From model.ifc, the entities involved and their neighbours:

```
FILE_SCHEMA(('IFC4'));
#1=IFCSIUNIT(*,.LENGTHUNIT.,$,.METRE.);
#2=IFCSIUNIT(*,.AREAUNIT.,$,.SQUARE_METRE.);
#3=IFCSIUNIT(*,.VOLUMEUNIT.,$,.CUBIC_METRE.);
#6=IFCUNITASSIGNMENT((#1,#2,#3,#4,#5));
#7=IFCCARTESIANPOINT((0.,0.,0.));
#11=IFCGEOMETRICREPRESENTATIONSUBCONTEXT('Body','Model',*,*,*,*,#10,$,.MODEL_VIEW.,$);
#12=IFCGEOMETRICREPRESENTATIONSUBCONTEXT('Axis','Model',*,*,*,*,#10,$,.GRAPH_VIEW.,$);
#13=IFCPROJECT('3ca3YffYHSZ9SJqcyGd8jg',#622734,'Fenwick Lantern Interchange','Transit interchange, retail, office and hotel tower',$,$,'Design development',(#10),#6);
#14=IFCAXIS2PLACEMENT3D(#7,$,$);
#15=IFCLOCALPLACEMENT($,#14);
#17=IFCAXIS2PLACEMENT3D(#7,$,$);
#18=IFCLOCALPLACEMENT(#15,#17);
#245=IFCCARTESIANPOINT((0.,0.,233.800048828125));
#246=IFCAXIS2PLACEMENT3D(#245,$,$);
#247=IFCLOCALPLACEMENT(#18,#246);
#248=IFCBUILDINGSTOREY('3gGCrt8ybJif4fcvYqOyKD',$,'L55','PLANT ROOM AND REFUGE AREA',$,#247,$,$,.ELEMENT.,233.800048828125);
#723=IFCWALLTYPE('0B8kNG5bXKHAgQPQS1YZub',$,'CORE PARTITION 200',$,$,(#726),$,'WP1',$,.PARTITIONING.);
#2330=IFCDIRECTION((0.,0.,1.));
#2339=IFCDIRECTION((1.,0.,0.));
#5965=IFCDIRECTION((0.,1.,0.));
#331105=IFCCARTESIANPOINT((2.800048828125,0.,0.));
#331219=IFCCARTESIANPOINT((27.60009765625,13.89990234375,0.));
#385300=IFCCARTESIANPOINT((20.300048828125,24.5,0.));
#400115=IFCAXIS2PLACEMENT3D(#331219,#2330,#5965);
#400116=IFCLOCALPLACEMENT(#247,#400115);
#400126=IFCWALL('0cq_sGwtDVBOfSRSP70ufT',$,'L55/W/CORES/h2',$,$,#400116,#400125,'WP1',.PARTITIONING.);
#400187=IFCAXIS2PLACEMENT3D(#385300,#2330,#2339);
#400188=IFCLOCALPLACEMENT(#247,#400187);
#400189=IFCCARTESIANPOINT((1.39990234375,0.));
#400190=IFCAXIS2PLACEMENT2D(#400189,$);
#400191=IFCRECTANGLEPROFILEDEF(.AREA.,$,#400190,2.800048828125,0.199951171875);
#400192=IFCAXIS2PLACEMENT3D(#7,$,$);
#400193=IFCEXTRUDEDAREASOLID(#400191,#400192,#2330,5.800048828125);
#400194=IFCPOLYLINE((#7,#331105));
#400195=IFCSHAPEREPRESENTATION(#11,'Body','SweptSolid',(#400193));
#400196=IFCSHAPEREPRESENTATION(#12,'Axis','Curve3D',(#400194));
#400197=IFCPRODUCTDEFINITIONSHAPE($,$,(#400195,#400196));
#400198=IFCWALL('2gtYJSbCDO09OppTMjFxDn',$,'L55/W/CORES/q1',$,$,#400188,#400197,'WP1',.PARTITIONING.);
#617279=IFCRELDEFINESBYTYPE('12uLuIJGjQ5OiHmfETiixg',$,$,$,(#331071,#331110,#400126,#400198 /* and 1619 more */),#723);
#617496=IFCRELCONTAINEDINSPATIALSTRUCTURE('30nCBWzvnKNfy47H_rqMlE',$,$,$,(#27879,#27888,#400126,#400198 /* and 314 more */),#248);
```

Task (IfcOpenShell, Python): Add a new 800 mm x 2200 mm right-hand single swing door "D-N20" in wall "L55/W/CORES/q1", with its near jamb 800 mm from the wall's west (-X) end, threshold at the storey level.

```python
import numpy as np
import ifcopenshell
import ifcopenshell.api.feature
import ifcopenshell.api.geometry
import ifcopenshell.api.root
import ifcopenshell.api.spatial
import ifcopenshell.geom
import ifcopenshell.util.element
import ifcopenshell.util.placement
import ifcopenshell.util.representation
import ifcopenshell.util.shape
import ifcopenshell.util.unit

model = ifcopenshell.open("model.ifc")
unit_scale = ifcopenshell.util.unit.calculate_unit_scale(model)
settings = ifcopenshell.geom.settings()


def volume(element):
    """Net volume in cubic metres, openings subtracted."""
    shape = ifcopenshell.geom.create_shape(settings, element)
    return ifcopenshell.util.shape.get_volume(shape.geometry)


wall = model.by_guid("2gtYJSbCDO09OppTMjFxDn")
storey = ifcopenshell.util.element.get_container(wall, ifc_class="IfcBuildingStorey")
context = ifcopenshell.util.representation.get_context(model, "Model", "Body", "MODEL_VIEW")
before = volume(wall)

width, height, from_end, sill = 0.8, 2.2, 0.8, 0.0  # metres

# The wall runs along its own X axis, and the end named is its -X end.
wall_shape = ifcopenshell.geom.create_shape(settings, wall)
x, y, z = ifcopenshell.util.shape.get_vertices(wall_shape.geometry).T
start = x.min() + from_end
face, thickness = float(y.min()), float(y.max() - y.min())
wall_matrix = ifcopenshell.util.placement.get_local_placement(wall.ObjectPlacement)
level = ifcopenshell.util.placement.get_local_placement(storey.ObjectPlacement)[2, 3]


def in_wall(x, y):
    """Placement at x, y metres in the wall's axes, at sill height."""
    matrix = wall_matrix.copy()
    matrix[:, 3] = wall_matrix @ np.array([x / unit_scale, y / unit_scale, 0.0, 1.0])
    matrix[2, 3] = level + sill / unit_scale
    return matrix


# Opening: a box that overshoots both wall faces by 50 mm.
opening = ifcopenshell.api.root.create_entity(model, ifc_class="IfcOpeningElement", predefined_type="OPENING")
box = ifcopenshell.api.geometry.add_wall_representation(
    model, context=context, length=width, height=height, thickness=thickness + 0.1
)
ifcopenshell.api.geometry.assign_representation(model, product=opening, representation=box)
ifcopenshell.api.geometry.edit_object_placement(model, product=opening, matrix=in_wall(start, face - 0.05), is_si=False)
ifcopenshell.api.feature.add_feature(model, feature=opening, element=wall)

door = ifcopenshell.api.root.create_entity(model, ifc_class="IfcDoor", name="D-N20", predefined_type="DOOR")
door.OverallWidth, door.OverallHeight = width / unit_scale, height / unit_scale
door.OperationType = "SINGLE_SWING_RIGHT"
body = ifcopenshell.api.geometry.add_door_representation(
    model,
    context=context,
    overall_width=door.OverallWidth,
    overall_height=door.OverallHeight,
    operation_type="SINGLE_SWING_RIGHT",
    lining_properties={"LiningDepth": thickness / unit_scale, "ThresholdDepth": thickness / unit_scale},
)
ifcopenshell.api.geometry.assign_representation(model, product=door, representation=body)
ifcopenshell.api.spatial.assign_container(model, products=[door], relating_structure=storey)
ifcopenshell.api.feature.add_filling(model, opening=opening, element=door)

# The lining spans the wall, so the door starts at the wall face.
ifcopenshell.api.geometry.edit_object_placement(model, product=door, matrix=in_wall(start, face), is_si=False)

after = volume(wall)

print(f"wall volume {before:.3f} -> {after:.3f} m3")

model.write("model_v2.ifc")
```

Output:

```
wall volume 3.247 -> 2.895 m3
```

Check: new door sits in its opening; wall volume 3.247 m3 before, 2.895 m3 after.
